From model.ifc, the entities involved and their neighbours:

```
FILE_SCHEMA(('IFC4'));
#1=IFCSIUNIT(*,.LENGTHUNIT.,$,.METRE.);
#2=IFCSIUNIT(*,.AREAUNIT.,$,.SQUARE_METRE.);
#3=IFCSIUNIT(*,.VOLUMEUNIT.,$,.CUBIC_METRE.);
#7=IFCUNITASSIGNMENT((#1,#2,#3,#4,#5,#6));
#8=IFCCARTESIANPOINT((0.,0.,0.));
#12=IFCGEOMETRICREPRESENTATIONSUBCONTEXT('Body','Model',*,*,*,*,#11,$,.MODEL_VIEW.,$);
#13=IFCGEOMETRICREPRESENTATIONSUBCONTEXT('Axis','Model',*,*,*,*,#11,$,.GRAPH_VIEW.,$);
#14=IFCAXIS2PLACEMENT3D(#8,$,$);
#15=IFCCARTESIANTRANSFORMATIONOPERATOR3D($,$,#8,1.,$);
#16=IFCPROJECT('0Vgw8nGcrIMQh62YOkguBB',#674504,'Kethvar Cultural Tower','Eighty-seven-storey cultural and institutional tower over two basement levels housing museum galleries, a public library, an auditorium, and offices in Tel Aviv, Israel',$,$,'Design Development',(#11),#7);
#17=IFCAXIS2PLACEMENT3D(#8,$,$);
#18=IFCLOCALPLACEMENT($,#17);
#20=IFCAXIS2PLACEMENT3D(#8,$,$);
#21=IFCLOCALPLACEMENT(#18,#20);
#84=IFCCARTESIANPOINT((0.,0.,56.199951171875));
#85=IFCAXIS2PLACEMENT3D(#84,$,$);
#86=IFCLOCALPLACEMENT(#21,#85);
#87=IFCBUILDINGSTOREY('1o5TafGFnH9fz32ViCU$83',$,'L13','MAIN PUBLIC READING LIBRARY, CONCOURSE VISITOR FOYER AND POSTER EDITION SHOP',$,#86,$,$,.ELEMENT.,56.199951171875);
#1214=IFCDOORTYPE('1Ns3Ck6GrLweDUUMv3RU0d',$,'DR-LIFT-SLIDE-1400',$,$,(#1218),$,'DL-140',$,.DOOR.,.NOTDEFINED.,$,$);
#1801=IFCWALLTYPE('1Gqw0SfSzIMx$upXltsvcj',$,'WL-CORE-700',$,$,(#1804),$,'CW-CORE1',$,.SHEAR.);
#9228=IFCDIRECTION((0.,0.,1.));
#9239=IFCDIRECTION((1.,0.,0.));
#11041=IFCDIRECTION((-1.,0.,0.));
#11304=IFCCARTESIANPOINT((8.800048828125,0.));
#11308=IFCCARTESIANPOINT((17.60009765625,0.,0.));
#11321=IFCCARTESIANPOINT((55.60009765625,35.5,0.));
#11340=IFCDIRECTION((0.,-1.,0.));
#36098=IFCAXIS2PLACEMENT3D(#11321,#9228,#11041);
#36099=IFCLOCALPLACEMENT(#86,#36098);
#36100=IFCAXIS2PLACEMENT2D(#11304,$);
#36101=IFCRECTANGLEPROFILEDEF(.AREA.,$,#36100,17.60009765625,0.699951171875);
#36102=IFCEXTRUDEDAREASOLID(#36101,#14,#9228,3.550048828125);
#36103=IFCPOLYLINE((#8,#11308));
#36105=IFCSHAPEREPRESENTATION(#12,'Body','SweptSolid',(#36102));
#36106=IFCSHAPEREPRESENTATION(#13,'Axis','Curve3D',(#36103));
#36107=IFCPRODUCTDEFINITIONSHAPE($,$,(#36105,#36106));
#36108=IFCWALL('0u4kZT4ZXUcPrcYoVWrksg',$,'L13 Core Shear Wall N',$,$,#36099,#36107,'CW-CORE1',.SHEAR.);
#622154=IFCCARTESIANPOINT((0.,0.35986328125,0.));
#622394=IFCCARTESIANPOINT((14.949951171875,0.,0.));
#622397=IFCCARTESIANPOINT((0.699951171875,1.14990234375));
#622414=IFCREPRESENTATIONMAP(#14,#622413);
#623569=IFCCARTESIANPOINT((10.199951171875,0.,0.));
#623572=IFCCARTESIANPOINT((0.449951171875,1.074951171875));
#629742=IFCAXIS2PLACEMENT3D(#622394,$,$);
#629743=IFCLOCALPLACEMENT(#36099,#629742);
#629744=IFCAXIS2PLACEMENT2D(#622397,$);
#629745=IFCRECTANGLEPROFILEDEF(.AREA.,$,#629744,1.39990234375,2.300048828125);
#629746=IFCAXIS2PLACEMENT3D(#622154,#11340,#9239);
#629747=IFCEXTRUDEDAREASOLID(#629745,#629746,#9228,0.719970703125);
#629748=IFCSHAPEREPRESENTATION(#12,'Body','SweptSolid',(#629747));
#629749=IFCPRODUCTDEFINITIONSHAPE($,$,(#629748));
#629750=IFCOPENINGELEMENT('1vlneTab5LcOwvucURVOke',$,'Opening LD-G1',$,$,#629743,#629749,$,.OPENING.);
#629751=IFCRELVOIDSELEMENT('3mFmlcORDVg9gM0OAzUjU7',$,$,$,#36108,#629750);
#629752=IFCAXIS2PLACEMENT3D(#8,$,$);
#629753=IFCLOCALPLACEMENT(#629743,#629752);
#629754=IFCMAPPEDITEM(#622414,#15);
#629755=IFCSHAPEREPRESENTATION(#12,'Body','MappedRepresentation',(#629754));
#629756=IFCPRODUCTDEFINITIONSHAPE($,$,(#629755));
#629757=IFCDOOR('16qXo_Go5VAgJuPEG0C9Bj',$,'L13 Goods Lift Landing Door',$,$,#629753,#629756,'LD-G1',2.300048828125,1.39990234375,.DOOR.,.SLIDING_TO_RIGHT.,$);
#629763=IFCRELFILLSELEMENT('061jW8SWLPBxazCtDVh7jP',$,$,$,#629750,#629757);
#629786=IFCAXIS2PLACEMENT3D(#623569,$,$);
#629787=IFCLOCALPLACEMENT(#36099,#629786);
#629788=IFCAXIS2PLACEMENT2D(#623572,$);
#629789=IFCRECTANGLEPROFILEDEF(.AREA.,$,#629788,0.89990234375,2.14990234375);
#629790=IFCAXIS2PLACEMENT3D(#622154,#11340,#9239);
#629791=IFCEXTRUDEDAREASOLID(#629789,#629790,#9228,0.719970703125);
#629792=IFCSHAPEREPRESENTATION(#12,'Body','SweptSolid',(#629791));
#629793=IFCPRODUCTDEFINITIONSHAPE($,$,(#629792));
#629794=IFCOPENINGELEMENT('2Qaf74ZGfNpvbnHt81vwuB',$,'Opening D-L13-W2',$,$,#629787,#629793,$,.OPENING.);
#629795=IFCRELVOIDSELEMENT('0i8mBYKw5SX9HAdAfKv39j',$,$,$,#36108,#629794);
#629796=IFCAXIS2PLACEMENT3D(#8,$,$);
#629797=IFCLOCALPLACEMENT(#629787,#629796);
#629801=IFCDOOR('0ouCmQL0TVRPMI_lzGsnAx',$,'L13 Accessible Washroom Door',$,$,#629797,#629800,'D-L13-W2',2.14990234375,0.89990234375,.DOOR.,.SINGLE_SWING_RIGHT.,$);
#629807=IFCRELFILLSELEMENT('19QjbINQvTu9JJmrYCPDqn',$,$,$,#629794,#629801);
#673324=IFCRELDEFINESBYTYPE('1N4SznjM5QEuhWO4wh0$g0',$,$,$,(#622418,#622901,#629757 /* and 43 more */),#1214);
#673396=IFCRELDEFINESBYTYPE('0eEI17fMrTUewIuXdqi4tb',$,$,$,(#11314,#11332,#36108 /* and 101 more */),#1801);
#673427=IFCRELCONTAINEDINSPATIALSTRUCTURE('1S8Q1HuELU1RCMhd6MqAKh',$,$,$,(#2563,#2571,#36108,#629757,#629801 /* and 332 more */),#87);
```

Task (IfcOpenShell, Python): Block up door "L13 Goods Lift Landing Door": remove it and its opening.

```python
import ifcopenshell
import ifcopenshell.api.feature
import ifcopenshell.api.root
import ifcopenshell.geom
import ifcopenshell.util.shape

model = ifcopenshell.open("model.ifc")
settings = ifcopenshell.geom.settings()


def volume(element):
    """Net volume in cubic metres, openings subtracted."""
    shape = ifcopenshell.geom.create_shape(settings, element)
    return ifcopenshell.util.shape.get_volume(shape.geometry)


door = model.by_guid("16qXo_Go5VAgJuPEG0C9Bj")
opening = door.FillsVoids[0].RelatingOpeningElement
wall = opening.VoidsElements[0].RelatingBuildingElement
before = volume(wall)

ifcopenshell.api.root.remove_product(model, product=door)
ifcopenshell.api.feature.remove_feature(model, feature=opening)

after = volume(wall)

print(f"wall volume {before:.3f} -> {after:.3f} m3")

model.write("model_updated.ifc")
```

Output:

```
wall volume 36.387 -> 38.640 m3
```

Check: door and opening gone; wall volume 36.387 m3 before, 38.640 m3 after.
